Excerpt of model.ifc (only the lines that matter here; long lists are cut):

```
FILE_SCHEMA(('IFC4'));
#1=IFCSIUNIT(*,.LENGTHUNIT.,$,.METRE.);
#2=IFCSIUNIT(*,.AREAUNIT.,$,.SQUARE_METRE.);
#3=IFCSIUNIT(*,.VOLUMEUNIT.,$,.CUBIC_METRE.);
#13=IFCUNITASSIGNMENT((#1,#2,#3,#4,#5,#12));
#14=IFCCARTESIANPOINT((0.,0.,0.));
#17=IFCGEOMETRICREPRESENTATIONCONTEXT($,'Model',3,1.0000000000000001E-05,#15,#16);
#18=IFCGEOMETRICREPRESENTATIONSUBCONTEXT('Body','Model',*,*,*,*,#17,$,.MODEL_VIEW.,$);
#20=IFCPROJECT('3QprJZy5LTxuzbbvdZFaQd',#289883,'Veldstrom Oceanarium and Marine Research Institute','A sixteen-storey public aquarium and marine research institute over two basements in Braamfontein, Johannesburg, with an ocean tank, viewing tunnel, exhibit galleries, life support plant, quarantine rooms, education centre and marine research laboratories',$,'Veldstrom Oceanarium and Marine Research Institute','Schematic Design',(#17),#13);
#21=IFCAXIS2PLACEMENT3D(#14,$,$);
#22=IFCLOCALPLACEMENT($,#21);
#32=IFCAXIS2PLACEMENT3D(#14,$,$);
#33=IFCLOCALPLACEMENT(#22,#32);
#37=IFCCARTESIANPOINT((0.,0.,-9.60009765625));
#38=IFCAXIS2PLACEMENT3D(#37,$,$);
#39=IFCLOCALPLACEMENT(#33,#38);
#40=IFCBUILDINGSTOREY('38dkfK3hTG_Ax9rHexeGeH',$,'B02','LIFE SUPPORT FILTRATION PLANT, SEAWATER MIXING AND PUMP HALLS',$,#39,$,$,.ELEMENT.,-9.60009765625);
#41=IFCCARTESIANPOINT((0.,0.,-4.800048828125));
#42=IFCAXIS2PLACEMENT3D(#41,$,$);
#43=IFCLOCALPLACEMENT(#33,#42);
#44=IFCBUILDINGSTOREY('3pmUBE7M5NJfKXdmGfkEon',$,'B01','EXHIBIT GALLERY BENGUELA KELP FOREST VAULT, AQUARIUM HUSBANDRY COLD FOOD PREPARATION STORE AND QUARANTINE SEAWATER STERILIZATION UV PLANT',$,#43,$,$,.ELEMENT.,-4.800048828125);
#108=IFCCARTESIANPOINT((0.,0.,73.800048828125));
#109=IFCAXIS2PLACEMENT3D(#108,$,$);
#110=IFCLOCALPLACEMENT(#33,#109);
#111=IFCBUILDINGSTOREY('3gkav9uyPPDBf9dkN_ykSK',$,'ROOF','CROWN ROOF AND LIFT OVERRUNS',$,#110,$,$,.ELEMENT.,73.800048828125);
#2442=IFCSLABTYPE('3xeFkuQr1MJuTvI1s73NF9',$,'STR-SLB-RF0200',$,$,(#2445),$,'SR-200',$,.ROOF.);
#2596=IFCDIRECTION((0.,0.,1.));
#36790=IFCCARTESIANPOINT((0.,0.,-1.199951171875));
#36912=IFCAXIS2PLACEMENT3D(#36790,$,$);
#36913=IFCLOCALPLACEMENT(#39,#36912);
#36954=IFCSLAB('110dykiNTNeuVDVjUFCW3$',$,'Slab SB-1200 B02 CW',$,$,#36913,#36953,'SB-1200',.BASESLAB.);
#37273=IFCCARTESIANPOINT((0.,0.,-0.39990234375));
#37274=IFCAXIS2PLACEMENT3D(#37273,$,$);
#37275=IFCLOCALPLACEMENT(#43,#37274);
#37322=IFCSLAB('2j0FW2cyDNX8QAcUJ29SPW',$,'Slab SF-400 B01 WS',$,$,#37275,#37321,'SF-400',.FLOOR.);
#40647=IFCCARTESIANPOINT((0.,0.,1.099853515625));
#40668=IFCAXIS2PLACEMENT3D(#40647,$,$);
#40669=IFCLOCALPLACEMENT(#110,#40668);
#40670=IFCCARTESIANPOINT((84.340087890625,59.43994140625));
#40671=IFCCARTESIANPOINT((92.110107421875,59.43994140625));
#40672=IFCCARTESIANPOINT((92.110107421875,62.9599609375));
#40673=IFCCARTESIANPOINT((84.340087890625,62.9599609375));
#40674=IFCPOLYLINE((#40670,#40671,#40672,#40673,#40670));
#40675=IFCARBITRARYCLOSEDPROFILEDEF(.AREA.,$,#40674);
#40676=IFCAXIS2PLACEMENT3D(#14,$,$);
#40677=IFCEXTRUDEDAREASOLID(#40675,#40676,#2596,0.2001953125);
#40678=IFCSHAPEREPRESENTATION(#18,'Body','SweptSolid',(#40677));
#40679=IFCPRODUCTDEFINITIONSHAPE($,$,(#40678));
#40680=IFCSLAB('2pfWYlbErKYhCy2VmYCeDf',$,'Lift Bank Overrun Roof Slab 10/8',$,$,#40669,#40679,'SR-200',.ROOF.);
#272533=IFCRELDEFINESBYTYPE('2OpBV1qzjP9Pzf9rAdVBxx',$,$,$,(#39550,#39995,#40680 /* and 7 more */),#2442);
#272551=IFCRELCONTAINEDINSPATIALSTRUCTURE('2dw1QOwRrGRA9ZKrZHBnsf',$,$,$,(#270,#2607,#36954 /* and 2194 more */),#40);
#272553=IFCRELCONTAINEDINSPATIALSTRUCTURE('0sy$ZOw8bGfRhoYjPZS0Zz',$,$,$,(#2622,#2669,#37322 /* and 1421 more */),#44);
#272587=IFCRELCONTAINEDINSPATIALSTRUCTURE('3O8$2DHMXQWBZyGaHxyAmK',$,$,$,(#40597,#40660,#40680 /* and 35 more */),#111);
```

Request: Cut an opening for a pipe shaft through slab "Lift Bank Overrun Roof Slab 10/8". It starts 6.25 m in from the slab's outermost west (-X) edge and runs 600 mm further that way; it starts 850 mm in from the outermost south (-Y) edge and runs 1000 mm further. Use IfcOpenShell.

```python
import numpy as np
import ifcopenshell
import ifcopenshell.api.feature
import ifcopenshell.api.geometry
import ifcopenshell.api.root
import ifcopenshell.geom
import ifcopenshell.util.placement
import ifcopenshell.util.representation
import ifcopenshell.util.shape
import ifcopenshell.util.unit

model = ifcopenshell.open("model.ifc")
unit_scale = ifcopenshell.util.unit.calculate_unit_scale(model)
settings = ifcopenshell.geom.settings()


def volume(element):
    """Net volume in cubic metres, openings subtracted."""
    shape = ifcopenshell.geom.create_shape(settings, element)
    return ifcopenshell.util.shape.get_volume(shape.geometry)


slab = model.by_guid("2pfWYlbErKYhCy2VmYCeDf")
before = volume(slab)

# Extent in the slab's own axes, in metres. The edges named are its -X and -Y sides.
slab_shape = ifcopenshell.geom.create_shape(settings, slab)
vertices = ifcopenshell.util.shape.get_vertices(slab_shape.geometry)
x_min, y_min, bottom = vertices.min(axis=0)
top = vertices[:, 2].max()

opening = ifcopenshell.api.root.create_entity(model, ifc_class="IfcOpeningElement", name="Pipe shaft opening", predefined_type="OPENING")
context = ifcopenshell.util.representation.get_context(model, "Model", "Body", "MODEL_VIEW")
width, depth = 0.6, 1
outline = [(0.0, 0.0), (width, 0.0), (width, depth), (0.0, depth), (0.0, 0.0)]
# Overshoot both faces by 50 mm so the cut is clean.
shape = ifcopenshell.api.geometry.add_slab_representation(
    model, context=context, depth=top - bottom + 0.1, polyline=outline
)
ifcopenshell.api.geometry.assign_representation(model, product=opening, representation=shape)

matrix = ifcopenshell.util.placement.get_local_placement(slab.ObjectPlacement)
matrix[:, 3] = matrix @ np.append(np.array([x_min + 6.25, y_min + 0.85, bottom - 0.05]) / unit_scale, 1.0)
ifcopenshell.api.geometry.edit_object_placement(model, product=opening, matrix=matrix, is_si=False)
ifcopenshell.api.feature.add_feature(model, feature=opening, element=slab)

after = volume(slab)

print(f"slab volume {before:.3f} -> {after:.3f} m3")

model.write("model_edited.ifc")
```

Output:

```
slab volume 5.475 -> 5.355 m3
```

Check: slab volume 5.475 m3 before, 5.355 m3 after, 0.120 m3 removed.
